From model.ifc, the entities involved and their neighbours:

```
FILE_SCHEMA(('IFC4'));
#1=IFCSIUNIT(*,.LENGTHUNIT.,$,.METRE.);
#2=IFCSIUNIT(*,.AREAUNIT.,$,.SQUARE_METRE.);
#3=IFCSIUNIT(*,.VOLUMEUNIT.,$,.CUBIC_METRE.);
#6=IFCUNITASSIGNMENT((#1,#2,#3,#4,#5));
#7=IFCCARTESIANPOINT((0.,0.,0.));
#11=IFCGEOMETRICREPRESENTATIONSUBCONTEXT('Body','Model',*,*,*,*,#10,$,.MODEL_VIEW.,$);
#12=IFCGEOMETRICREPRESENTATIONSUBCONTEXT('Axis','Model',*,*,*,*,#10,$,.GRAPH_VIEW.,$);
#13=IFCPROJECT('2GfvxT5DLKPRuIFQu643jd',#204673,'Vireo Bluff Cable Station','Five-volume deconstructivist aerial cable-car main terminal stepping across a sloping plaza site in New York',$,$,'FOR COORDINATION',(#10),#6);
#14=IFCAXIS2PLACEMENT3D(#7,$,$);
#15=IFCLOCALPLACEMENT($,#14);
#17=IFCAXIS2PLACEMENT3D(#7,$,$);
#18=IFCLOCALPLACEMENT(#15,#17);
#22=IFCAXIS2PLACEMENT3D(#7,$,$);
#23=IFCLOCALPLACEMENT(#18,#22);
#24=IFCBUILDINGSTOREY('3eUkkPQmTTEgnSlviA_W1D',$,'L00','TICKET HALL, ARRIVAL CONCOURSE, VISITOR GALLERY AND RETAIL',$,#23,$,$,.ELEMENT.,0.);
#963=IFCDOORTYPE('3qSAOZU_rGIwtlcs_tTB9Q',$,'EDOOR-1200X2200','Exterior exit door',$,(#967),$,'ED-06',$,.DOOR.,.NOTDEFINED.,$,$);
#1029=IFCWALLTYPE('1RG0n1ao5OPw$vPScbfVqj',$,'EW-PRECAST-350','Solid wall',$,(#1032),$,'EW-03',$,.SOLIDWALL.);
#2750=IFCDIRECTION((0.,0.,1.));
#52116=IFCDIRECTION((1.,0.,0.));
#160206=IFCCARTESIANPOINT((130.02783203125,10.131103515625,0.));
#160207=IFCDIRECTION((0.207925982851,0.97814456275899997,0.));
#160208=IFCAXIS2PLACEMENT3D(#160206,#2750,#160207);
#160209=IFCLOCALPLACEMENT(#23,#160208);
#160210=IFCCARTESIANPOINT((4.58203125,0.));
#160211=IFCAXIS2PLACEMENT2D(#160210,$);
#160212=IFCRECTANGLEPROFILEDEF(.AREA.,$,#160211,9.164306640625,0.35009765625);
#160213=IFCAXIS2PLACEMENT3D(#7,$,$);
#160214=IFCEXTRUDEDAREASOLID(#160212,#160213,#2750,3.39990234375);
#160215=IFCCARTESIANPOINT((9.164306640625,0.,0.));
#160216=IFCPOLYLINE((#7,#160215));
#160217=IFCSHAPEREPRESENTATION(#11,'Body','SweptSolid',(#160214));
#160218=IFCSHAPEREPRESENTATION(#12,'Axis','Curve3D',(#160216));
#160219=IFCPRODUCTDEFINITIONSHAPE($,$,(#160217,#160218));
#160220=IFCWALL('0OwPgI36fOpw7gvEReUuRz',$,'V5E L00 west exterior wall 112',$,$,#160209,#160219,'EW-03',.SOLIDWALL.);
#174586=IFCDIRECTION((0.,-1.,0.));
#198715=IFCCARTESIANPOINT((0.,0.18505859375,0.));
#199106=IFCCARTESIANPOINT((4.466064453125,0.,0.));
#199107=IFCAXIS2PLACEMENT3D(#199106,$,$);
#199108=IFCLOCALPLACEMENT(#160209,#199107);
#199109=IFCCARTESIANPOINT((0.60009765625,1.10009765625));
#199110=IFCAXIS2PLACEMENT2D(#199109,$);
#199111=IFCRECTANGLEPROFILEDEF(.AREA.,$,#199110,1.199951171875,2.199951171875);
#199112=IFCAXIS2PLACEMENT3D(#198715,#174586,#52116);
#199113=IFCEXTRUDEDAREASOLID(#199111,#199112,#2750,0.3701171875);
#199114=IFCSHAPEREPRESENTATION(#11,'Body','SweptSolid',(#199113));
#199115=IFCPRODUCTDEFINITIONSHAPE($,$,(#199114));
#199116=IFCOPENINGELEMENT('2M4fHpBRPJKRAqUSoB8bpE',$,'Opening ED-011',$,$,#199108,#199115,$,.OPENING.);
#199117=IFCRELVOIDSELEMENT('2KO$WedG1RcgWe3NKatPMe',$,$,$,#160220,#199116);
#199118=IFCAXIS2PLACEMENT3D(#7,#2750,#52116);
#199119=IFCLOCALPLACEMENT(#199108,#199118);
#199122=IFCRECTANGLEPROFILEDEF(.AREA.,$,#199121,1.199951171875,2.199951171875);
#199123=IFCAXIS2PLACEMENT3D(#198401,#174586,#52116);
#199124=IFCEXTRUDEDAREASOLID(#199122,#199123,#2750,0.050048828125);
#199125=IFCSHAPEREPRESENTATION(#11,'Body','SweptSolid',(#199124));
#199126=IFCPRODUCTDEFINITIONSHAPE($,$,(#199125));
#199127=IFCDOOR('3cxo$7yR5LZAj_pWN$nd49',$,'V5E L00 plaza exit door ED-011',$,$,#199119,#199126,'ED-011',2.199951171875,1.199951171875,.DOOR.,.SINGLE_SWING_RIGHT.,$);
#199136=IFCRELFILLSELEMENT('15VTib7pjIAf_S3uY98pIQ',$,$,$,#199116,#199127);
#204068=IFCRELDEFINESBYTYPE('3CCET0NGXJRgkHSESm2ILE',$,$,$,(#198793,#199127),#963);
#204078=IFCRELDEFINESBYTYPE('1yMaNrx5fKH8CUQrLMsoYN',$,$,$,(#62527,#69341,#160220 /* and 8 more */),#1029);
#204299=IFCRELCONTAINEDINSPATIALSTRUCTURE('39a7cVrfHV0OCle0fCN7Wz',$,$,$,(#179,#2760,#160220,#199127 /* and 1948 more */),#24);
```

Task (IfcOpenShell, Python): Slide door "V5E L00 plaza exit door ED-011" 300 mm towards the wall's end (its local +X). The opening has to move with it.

```python
import ifcopenshell
import ifcopenshell.api.geometry
import ifcopenshell.util.placement
import ifcopenshell.util.unit

model = ifcopenshell.open("model.ifc")
unit_scale = ifcopenshell.util.unit.calculate_unit_scale(model)

door = model.by_id(199127)
opening = door.FillsVoids[0].RelatingOpeningElement
wall = opening.VoidsElements[0].RelatingBuildingElement

wall_matrix = ifcopenshell.util.placement.get_local_placement(wall.ObjectPlacement)
shift = wall_matrix[:3, 0] * 0.3 / unit_scale
before = ifcopenshell.util.placement.get_local_placement(door.ObjectPlacement)[:3, 3].copy()

# The door is placed relative to its opening, so it follows when the opening moves.
matrix = ifcopenshell.util.placement.get_local_placement(opening.ObjectPlacement)
matrix[:3, 3] += shift
ifcopenshell.api.geometry.edit_object_placement(
    model, product=opening, matrix=matrix, is_si=False, should_transform_children=True
)

after = ifcopenshell.util.placement.get_local_placement(door.ObjectPlacement)[:3, 3]
print("door moved by", (after - before).round(3) + 0.0)

model.write("model_v2.ifc")
```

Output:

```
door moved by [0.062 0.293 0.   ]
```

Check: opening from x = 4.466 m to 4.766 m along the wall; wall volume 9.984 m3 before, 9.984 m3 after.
